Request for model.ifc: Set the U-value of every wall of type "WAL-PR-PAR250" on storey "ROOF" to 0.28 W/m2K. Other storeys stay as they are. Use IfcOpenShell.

First a look at what the model holds.

```python
import ifcopenshell
import ifcopenshell.util.element

model = ifcopenshell.open("model.ifc")
print(model.schema)
storey = next(s for s in model.by_type("IfcBuildingStorey") if s.Name == "ROOF")
walls = [e for e in ifcopenshell.util.element.get_decomposition(storey) if e.is_a("IfcWall")]
seen = {}
for e in walls:
    element_type = ifcopenshell.util.element.get_type(e)
    key = (element_type.Name if element_type != e and element_type else None, ifcopenshell.util.element.get_pset(e, "Pset_WallCommon", "ThermalTransmittance"))
    seen[key] = seen.get(key, 0) + 1
for (name, value), count in sorted(seen.items(), key=str):
    print(count, "x", name, "|", value)
```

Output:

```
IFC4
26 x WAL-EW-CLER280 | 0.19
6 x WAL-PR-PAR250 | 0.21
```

```python
import ifcopenshell
import ifcopenshell.api.pset
import ifcopenshell.util.element

model = ifcopenshell.open("model.ifc")

storey = next(s for s in model.by_type("IfcBuildingStorey") if s.Name == "ROOF")
walls = [e for e in ifcopenshell.util.element.get_decomposition(storey) if e.is_a("IfcWall")]

count = 0
for e in walls:
    element_type = ifcopenshell.util.element.get_type(e)
    if element_type in (None, e) or element_type.Name != "WAL-PR-PAR250":
        continue
    # add_pset returns the element's existing set when there is one.
    pset = ifcopenshell.api.pset.add_pset(model, product=e, name="Pset_WallCommon")
    ifcopenshell.api.pset.edit_pset(model, pset=pset, properties={"ThermalTransmittance": 0.28})
    count += 1

print(count, "walls updated")

model.write("model_rev.ifc")
```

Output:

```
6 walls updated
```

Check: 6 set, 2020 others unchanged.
